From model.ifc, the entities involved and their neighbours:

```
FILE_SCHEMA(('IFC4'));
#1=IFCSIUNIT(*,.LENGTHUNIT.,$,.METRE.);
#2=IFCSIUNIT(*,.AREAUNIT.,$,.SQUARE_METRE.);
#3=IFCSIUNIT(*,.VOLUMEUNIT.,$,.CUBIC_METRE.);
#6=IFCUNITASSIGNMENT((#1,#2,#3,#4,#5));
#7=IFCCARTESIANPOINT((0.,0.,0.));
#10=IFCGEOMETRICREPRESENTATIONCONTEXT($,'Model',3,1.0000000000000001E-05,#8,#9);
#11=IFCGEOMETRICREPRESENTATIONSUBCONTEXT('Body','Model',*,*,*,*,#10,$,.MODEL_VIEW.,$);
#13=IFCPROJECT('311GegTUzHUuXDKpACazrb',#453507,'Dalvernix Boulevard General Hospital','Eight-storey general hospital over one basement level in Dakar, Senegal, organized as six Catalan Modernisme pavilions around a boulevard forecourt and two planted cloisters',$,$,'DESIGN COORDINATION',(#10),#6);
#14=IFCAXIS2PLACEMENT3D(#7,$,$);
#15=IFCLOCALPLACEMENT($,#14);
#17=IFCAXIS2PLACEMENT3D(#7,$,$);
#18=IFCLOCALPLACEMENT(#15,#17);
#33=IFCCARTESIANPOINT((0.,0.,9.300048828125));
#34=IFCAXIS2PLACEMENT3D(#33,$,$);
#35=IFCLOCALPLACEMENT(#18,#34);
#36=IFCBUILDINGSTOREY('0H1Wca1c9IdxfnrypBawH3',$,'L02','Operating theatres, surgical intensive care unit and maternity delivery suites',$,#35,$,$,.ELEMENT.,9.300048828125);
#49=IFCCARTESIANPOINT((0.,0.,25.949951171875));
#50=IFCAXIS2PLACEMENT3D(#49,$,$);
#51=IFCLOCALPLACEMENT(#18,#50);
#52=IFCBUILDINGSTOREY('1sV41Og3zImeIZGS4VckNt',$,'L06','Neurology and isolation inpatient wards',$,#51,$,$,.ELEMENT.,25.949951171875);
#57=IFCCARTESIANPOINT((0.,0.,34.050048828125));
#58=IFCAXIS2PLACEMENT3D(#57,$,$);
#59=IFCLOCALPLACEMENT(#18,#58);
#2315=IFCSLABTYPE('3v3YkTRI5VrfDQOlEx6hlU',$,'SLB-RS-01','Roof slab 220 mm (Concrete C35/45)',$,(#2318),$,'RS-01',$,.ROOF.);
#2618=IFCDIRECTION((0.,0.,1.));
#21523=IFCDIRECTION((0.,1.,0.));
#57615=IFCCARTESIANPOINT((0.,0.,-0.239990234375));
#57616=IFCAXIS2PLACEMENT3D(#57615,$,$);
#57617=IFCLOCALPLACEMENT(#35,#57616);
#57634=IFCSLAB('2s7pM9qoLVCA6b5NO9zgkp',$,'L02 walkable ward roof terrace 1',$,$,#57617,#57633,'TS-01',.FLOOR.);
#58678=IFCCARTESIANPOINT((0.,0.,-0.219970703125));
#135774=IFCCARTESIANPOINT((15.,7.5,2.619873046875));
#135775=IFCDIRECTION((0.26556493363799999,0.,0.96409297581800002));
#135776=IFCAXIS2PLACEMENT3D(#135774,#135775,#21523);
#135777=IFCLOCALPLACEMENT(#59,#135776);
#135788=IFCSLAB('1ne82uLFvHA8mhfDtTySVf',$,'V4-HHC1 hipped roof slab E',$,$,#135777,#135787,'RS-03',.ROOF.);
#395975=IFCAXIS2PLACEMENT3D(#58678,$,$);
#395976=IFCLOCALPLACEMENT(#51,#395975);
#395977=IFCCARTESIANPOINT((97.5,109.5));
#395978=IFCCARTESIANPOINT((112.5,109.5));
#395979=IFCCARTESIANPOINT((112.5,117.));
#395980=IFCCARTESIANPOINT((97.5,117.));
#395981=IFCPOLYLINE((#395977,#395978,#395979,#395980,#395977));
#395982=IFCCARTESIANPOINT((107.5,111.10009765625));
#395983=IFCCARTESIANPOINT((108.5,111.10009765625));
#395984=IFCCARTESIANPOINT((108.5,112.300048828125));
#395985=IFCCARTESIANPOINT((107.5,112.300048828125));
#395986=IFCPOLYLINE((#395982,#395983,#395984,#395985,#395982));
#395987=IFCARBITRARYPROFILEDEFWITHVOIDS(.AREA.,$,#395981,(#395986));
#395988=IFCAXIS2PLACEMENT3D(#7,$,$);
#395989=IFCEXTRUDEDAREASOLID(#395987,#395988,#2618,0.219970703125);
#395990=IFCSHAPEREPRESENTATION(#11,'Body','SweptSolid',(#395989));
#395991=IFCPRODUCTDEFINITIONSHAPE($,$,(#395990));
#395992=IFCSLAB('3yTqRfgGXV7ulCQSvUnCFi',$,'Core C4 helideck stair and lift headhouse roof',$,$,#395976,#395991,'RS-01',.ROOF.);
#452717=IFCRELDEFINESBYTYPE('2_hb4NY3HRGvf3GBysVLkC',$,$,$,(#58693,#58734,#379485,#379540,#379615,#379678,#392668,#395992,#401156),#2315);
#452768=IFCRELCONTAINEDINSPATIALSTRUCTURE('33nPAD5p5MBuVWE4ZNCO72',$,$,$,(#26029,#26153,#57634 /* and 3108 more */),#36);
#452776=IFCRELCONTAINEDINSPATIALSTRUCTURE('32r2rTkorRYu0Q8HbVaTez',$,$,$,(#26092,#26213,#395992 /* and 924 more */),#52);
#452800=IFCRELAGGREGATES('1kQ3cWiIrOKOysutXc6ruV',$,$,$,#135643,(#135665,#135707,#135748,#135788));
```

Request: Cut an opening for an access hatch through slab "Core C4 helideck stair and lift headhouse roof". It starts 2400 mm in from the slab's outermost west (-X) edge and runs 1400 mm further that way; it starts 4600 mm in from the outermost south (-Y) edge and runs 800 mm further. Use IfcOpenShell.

```python
import numpy as np
import ifcopenshell
import ifcopenshell.api.feature
import ifcopenshell.api.geometry
import ifcopenshell.api.root
import ifcopenshell.geom
import ifcopenshell.util.placement
import ifcopenshell.util.representation
import ifcopenshell.util.shape
import ifcopenshell.util.unit

model = ifcopenshell.open("model.ifc")
unit_scale = ifcopenshell.util.unit.calculate_unit_scale(model)
settings = ifcopenshell.geom.settings()


def volume(element):
    """Net volume in cubic metres, openings subtracted."""
    shape = ifcopenshell.geom.create_shape(settings, element)
    return ifcopenshell.util.shape.get_volume(shape.geometry)


slab = model.by_guid("3yTqRfgGXV7ulCQSvUnCFi")
before = volume(slab)

# Extent in the slab's own axes, in metres. The edges named are its -X and -Y sides.
slab_shape = ifcopenshell.geom.create_shape(settings, slab)
vertices = ifcopenshell.util.shape.get_vertices(slab_shape.geometry)
x_min, y_min, bottom = vertices.min(axis=0)
top = vertices[:, 2].max()

opening = ifcopenshell.api.root.create_entity(model, ifc_class="IfcOpeningElement", name="Access hatch opening", predefined_type="OPENING")
context = ifcopenshell.util.representation.get_context(model, "Model", "Body", "MODEL_VIEW")
width, depth = 1.4, 0.8
outline = [(0.0, 0.0), (width, 0.0), (width, depth), (0.0, depth), (0.0, 0.0)]
# Overshoot both faces by 50 mm so the cut is clean.
shape = ifcopenshell.api.geometry.add_slab_representation(
    model, context=context, depth=top - bottom + 0.1, polyline=outline
)
ifcopenshell.api.geometry.assign_representation(model, product=opening, representation=shape)

matrix = ifcopenshell.util.placement.get_local_placement(slab.ObjectPlacement)
matrix[:, 3] = matrix @ np.append(np.array([x_min + 2.4, y_min + 4.6, bottom - 0.05]) / unit_scale, 1.0)
ifcopenshell.api.geometry.edit_object_placement(model, product=opening, matrix=matrix, is_si=False)
ifcopenshell.api.feature.add_feature(model, feature=opening, element=slab)

after = volume(slab)

print(f"slab volume {before:.3f} -> {after:.3f} m3")

model.write("model_edited.ifc")
```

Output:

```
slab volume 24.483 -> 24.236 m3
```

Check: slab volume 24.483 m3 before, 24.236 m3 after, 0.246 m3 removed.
